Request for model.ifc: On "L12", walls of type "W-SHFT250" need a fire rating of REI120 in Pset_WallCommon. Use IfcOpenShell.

First a look at what the model holds.

```python
import ifcopenshell
import ifcopenshell.util.element

model = ifcopenshell.open("model.ifc")
print(model.schema)
storey = next(s for s in model.by_type("IfcBuildingStorey") if s.Name == "L12")
walls = [e for e in ifcopenshell.util.element.get_decomposition(storey) if e.is_a("IfcWall")]
seen = {}
for e in walls:
    element_type = ifcopenshell.util.element.get_type(e)
    key = (element_type.Name if element_type != e and element_type else None, ifcopenshell.util.element.get_pset(e, "Pset_WallCommon", "FireRating"))
    seen[key] = seen.get(key, 0) + 1
for (name, value), count in sorted(seen.items(), key=str):
    print(count, "x", name, "|", value)
```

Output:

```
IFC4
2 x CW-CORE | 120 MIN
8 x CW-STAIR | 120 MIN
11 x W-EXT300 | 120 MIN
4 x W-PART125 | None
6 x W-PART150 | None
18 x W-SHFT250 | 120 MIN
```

```python
import ifcopenshell
import ifcopenshell.api.pset
import ifcopenshell.util.element

model = ifcopenshell.open("model.ifc")

storey = next(s for s in model.by_type("IfcBuildingStorey") if s.Name == "L12")
walls = [e for e in ifcopenshell.util.element.get_decomposition(storey) if e.is_a("IfcWall")]

count = 0
for e in walls:
    element_type = ifcopenshell.util.element.get_type(e)
    if element_type in (None, e) or element_type.Name != "W-SHFT250":
        continue
    # add_pset returns the element's existing set when there is one.
    pset = ifcopenshell.api.pset.add_pset(model, product=e, name="Pset_WallCommon")
    ifcopenshell.api.pset.edit_pset(model, pset=pset, properties={"FireRating": "REI120"})
    count += 1

print(count, "walls updated")

model.write("model-out.ifc")
```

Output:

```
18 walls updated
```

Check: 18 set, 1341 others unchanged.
